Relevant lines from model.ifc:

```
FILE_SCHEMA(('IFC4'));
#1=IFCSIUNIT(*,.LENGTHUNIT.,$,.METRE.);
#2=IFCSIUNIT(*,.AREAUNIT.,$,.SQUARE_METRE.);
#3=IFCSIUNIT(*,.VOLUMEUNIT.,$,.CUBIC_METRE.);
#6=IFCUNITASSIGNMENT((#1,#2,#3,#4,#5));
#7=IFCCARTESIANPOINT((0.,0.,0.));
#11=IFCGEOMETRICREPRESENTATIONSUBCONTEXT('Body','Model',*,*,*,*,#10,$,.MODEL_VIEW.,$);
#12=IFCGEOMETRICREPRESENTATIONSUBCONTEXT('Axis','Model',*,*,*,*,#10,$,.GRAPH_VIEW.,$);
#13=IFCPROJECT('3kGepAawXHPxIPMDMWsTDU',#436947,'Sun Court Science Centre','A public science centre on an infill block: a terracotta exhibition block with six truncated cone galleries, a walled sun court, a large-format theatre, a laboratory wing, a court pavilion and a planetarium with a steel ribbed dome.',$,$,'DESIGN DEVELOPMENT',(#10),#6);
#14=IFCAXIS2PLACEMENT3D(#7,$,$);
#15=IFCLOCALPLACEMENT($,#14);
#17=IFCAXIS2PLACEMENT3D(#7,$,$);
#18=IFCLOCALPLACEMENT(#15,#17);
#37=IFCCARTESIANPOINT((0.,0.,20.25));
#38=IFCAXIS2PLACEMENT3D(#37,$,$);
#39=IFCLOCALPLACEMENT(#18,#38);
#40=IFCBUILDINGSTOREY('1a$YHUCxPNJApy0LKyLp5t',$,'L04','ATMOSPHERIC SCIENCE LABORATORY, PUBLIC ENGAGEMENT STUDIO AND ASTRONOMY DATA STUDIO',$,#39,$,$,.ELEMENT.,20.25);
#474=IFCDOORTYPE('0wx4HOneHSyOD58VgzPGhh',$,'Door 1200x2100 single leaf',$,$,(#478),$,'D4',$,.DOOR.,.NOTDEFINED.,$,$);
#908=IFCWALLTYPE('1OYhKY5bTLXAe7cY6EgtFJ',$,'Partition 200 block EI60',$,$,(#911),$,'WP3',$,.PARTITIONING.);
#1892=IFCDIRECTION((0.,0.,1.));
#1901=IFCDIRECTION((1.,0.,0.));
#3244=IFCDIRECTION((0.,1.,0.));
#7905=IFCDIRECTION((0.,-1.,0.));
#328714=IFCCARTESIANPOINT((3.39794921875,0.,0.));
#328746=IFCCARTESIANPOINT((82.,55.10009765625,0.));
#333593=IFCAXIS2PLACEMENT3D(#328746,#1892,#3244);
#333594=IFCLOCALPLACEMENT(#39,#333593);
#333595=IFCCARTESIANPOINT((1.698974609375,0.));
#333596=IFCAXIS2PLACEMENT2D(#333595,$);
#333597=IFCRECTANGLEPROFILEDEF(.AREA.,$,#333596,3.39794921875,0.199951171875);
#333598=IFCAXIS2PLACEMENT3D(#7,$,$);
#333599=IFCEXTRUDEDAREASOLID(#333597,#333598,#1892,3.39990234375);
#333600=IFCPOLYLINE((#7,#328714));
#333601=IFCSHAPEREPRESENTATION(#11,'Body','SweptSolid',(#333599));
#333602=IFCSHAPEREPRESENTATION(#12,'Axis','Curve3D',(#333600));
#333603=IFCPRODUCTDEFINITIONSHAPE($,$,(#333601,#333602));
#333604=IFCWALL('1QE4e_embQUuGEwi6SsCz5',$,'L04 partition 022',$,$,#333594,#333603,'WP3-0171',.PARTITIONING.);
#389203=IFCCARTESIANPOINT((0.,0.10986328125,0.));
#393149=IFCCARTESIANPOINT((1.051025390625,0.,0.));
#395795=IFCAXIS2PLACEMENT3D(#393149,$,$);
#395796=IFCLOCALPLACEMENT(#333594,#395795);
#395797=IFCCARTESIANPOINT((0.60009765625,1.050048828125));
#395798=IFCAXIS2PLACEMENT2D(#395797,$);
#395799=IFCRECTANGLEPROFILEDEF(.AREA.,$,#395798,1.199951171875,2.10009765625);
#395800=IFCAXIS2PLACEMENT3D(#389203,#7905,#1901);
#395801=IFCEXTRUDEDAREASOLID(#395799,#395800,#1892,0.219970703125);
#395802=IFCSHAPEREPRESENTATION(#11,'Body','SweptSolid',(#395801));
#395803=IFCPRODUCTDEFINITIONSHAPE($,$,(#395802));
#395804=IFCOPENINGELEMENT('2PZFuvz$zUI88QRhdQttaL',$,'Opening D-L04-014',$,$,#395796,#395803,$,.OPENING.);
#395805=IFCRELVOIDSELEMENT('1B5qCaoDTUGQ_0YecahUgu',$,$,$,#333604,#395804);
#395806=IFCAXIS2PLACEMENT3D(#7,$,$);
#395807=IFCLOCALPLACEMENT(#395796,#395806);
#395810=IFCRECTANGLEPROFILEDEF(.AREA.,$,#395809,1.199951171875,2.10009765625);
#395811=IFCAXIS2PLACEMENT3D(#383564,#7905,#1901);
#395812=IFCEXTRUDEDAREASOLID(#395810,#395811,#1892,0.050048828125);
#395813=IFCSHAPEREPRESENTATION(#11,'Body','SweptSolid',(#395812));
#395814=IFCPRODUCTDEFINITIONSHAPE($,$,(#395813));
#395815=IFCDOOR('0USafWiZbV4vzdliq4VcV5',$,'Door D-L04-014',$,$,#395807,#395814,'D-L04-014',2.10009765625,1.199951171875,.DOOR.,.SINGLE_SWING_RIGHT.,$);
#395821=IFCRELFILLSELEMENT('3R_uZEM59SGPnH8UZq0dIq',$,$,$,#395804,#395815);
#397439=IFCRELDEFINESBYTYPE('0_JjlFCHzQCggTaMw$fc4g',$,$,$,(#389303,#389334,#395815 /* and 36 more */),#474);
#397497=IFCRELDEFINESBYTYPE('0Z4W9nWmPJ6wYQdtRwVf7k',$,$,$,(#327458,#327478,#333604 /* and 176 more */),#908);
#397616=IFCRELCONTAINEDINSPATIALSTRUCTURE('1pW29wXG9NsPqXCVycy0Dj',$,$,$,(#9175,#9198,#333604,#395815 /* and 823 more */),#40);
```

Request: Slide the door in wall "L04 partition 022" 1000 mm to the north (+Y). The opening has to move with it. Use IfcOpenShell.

```python
import ifcopenshell
import ifcopenshell.api.geometry
import ifcopenshell.util.placement
import ifcopenshell.util.unit

model = ifcopenshell.open("model.ifc")
unit_scale = ifcopenshell.util.unit.calculate_unit_scale(model)

door = model.by_guid("0USafWiZbV4vzdliq4VcV5")
opening = door.FillsVoids[0].RelatingOpeningElement
wall = opening.VoidsElements[0].RelatingBuildingElement

wall_matrix = ifcopenshell.util.placement.get_local_placement(wall.ObjectPlacement)
shift = wall_matrix[:3, 0] * 1 / unit_scale
before = ifcopenshell.util.placement.get_local_placement(door.ObjectPlacement)[:3, 3].copy()

# The door is placed relative to its opening, so it follows when the opening moves.
matrix = ifcopenshell.util.placement.get_local_placement(opening.ObjectPlacement)
matrix[:3, 3] += shift
ifcopenshell.api.geometry.edit_object_placement(
    model, product=opening, matrix=matrix, is_si=False, should_transform_children=True
)

after = ifcopenshell.util.placement.get_local_placement(door.ObjectPlacement)[:3, 3]
print("door moved by", (after - before).round(3) + 0.0)

model.write("model_edited.ifc")
```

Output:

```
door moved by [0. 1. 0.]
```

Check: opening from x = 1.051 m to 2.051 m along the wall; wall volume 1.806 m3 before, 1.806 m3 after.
